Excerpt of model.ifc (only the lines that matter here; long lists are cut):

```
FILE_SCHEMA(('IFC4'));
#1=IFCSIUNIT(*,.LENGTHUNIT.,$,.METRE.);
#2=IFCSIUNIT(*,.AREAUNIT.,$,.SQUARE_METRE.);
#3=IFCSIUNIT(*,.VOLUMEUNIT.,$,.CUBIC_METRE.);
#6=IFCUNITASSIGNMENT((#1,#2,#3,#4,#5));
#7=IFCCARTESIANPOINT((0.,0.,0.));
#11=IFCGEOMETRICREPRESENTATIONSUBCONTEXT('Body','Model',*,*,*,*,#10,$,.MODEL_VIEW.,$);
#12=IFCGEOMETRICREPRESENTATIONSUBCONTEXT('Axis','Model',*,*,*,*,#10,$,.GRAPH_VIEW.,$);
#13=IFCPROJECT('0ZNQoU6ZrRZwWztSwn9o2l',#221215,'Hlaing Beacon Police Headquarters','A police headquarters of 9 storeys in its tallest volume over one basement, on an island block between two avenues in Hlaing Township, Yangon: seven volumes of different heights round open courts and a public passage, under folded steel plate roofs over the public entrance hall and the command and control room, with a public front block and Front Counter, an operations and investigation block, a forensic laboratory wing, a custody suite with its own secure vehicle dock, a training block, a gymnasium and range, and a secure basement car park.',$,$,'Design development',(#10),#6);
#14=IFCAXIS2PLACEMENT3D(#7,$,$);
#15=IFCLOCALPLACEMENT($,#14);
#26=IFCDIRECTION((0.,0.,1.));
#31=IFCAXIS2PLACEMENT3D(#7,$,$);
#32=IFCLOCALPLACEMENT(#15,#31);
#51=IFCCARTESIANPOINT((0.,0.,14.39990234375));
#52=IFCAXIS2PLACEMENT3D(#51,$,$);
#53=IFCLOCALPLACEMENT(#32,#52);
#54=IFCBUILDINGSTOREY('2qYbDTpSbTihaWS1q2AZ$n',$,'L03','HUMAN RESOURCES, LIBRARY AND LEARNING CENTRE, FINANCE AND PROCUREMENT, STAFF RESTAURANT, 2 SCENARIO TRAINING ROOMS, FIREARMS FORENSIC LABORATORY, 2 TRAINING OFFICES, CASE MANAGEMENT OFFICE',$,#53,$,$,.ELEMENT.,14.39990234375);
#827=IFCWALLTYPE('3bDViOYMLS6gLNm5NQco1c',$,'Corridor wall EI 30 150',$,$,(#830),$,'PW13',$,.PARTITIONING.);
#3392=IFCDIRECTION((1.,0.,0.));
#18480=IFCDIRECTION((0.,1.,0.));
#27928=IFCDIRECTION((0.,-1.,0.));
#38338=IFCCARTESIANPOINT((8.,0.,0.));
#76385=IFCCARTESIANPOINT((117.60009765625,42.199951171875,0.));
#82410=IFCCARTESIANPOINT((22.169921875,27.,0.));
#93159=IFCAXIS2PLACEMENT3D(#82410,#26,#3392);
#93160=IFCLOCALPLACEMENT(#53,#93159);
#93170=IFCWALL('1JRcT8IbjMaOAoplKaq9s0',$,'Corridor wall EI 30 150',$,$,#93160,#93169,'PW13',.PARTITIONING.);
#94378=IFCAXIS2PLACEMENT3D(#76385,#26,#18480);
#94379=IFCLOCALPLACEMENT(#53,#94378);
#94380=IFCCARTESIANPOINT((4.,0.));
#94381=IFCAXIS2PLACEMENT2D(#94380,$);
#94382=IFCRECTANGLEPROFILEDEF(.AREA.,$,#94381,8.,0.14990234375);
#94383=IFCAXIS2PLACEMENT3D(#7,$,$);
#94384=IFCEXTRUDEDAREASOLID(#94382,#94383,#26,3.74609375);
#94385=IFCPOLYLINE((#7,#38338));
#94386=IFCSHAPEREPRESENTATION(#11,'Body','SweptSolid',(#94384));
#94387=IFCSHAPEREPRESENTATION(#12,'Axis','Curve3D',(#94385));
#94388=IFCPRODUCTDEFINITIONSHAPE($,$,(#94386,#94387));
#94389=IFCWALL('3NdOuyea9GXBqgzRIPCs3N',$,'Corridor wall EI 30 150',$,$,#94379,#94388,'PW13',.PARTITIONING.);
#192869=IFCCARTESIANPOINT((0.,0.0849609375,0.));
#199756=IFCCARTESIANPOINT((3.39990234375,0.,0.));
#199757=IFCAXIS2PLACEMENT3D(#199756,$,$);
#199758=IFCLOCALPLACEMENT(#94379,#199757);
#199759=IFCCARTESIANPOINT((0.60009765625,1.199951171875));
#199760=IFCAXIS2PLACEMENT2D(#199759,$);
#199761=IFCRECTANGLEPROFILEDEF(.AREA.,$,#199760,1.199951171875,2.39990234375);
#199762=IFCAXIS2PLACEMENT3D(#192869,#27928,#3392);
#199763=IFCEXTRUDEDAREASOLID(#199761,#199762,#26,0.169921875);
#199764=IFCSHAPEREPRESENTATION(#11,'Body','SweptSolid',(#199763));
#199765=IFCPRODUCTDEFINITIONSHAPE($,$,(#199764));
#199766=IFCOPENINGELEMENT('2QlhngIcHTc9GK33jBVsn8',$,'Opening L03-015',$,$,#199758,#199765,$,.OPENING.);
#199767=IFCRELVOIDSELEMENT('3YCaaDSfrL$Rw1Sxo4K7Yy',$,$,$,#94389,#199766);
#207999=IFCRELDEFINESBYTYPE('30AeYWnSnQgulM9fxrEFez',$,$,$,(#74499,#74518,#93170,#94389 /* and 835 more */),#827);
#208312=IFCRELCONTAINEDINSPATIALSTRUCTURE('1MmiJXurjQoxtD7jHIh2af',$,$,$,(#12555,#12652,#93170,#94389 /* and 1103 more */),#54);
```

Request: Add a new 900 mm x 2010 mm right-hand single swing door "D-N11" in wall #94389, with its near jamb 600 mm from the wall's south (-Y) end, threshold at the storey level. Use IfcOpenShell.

```python
import numpy as np
import ifcopenshell
import ifcopenshell.api.feature
import ifcopenshell.api.geometry
import ifcopenshell.api.root
import ifcopenshell.api.spatial
import ifcopenshell.geom
import ifcopenshell.util.element
import ifcopenshell.util.placement
import ifcopenshell.util.representation
import ifcopenshell.util.shape
import ifcopenshell.util.unit

model = ifcopenshell.open("model.ifc")
unit_scale = ifcopenshell.util.unit.calculate_unit_scale(model)
settings = ifcopenshell.geom.settings()


def volume(element):
    """Net volume in cubic metres, openings subtracted."""
    shape = ifcopenshell.geom.create_shape(settings, element)
    return ifcopenshell.util.shape.get_volume(shape.geometry)


wall = model.by_id(94389)
storey = ifcopenshell.util.element.get_container(wall, ifc_class="IfcBuildingStorey")
context = ifcopenshell.util.representation.get_context(model, "Model", "Body", "MODEL_VIEW")
before = volume(wall)

width, height, from_end, sill = 0.9, 2.01, 0.6, 0.0  # metres

# The wall runs along its own X axis, and the end named is its -X end.
wall_shape = ifcopenshell.geom.create_shape(settings, wall)
x, y, z = ifcopenshell.util.shape.get_vertices(wall_shape.geometry).T
start = x.min() + from_end
face, thickness = float(y.min()), float(y.max() - y.min())
wall_matrix = ifcopenshell.util.placement.get_local_placement(wall.ObjectPlacement)
level = ifcopenshell.util.placement.get_local_placement(storey.ObjectPlacement)[2, 3]


def in_wall(x, y):
    """Placement at x, y metres in the wall's axes, at sill height."""
    matrix = wall_matrix.copy()
    matrix[:, 3] = wall_matrix @ np.array([x / unit_scale, y / unit_scale, 0.0, 1.0])
    matrix[2, 3] = level + sill / unit_scale
    return matrix


# Opening: a box that overshoots both wall faces by 50 mm.
opening = ifcopenshell.api.root.create_entity(model, ifc_class="IfcOpeningElement", predefined_type="OPENING")
box = ifcopenshell.api.geometry.add_wall_representation(
    model, context=context, length=width, height=height, thickness=thickness + 0.1
)
ifcopenshell.api.geometry.assign_representation(model, product=opening, representation=box)
ifcopenshell.api.geometry.edit_object_placement(model, product=opening, matrix=in_wall(start, face - 0.05), is_si=False)
ifcopenshell.api.feature.add_feature(model, feature=opening, element=wall)

door = ifcopenshell.api.root.create_entity(model, ifc_class="IfcDoor", name="D-N11", predefined_type="DOOR")
door.OverallWidth, door.OverallHeight = width / unit_scale, height / unit_scale
door.OperationType = "SINGLE_SWING_RIGHT"
body = ifcopenshell.api.geometry.add_door_representation(
    model,
    context=context,
    overall_width=door.OverallWidth,
    overall_height=door.OverallHeight,
    operation_type="SINGLE_SWING_RIGHT",
    lining_properties={"LiningDepth": thickness / unit_scale, "ThresholdDepth": thickness / unit_scale},
)
ifcopenshell.api.geometry.assign_representation(model, product=door, representation=body)
ifcopenshell.api.spatial.assign_container(model, products=[door], relating_structure=storey)
ifcopenshell.api.feature.add_filling(model, opening=opening, element=door)

# The lining spans the wall, so the door starts at the wall face.
ifcopenshell.api.geometry.edit_object_placement(model, product=door, matrix=in_wall(start, face), is_si=False)

after = volume(wall)

print(f"wall volume {before:.3f} -> {after:.3f} m3")

model.write("model_v2.ifc")
```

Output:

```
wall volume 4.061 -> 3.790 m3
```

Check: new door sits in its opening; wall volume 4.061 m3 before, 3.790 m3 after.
